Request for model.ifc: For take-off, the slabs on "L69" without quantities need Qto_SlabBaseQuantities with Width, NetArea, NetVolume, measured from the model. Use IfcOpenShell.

First a look at what the model holds.

```python
import ifcopenshell
import ifcopenshell.util.element
import ifcopenshell.util.unit

model = ifcopenshell.open("model.ifc")
print(model.schema)
for unit_type in ("LENGTHUNIT", "AREAUNIT", "VOLUMEUNIT"):
    print(unit_type, ifcopenshell.util.unit.calculate_unit_scale(model, unit_type))
storey = next(s for s in model.by_type("IfcBuildingStorey") if s.Name == "L69")
slabs = [e for e in ifcopenshell.util.element.get_decomposition(storey) if e.is_a("IfcSlab")]
for e in sorted(slabs, key=lambda e: e.id()):
    print(e.id(), e.is_a(), e.Name, list(ifcopenshell.util.element.get_psets(e, qtos_only=True)), sep=" | ")
```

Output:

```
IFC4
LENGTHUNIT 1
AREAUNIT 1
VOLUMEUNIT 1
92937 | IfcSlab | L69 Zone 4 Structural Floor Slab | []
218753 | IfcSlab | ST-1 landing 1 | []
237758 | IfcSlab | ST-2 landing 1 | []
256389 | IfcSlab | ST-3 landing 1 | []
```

```python
import ifcopenshell
import ifcopenshell.api.pset
import ifcopenshell.geom
import ifcopenshell.util.element
import ifcopenshell.util.shape
import ifcopenshell.util.unit

model = ifcopenshell.open("model.ifc")
unit_scale = ifcopenshell.util.unit.calculate_unit_scale(model)
area_scale = ifcopenshell.util.unit.calculate_unit_scale(model, "AREAUNIT")
volume_scale = ifcopenshell.util.unit.calculate_unit_scale(model, "VOLUMEUNIT")
settings = ifcopenshell.geom.settings()

storey = next(s for s in model.by_type("IfcBuildingStorey") if s.Name == "L69")
slabs = [e for e in ifcopenshell.util.element.get_decomposition(storey) if e.is_a("IfcSlab")]

for e in sorted(slabs, key=lambda e: e.id()):
    if ifcopenshell.util.element.get_psets(e, qtos_only=True, should_inherit=False):
        continue
    # Geometry comes back in metres, in the element's own axes.
    shape = ifcopenshell.geom.create_shape(settings, e)
    values = {
        "Width": ifcopenshell.util.shape.get_z(shape.geometry) / unit_scale,
        "NetArea": ifcopenshell.util.shape.get_footprint_area(shape.geometry) / area_scale,
        "NetVolume": ifcopenshell.util.shape.get_volume(shape.geometry) / volume_scale,
    }
    qto = ifcopenshell.api.pset.add_qto(model, product=e, name="Qto_SlabBaseQuantities")
    ifcopenshell.api.pset.edit_qto(model, qto=qto, properties=values)
    print(e.id(), {k: round(v, 3) for k, v in values.items()})

model.write("model_rev.ifc")
```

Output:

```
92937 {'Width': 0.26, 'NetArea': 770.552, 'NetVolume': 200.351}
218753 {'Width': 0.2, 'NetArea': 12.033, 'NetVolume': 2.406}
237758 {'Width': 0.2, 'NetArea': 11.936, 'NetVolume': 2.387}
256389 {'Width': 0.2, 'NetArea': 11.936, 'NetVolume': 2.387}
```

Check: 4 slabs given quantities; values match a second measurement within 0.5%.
